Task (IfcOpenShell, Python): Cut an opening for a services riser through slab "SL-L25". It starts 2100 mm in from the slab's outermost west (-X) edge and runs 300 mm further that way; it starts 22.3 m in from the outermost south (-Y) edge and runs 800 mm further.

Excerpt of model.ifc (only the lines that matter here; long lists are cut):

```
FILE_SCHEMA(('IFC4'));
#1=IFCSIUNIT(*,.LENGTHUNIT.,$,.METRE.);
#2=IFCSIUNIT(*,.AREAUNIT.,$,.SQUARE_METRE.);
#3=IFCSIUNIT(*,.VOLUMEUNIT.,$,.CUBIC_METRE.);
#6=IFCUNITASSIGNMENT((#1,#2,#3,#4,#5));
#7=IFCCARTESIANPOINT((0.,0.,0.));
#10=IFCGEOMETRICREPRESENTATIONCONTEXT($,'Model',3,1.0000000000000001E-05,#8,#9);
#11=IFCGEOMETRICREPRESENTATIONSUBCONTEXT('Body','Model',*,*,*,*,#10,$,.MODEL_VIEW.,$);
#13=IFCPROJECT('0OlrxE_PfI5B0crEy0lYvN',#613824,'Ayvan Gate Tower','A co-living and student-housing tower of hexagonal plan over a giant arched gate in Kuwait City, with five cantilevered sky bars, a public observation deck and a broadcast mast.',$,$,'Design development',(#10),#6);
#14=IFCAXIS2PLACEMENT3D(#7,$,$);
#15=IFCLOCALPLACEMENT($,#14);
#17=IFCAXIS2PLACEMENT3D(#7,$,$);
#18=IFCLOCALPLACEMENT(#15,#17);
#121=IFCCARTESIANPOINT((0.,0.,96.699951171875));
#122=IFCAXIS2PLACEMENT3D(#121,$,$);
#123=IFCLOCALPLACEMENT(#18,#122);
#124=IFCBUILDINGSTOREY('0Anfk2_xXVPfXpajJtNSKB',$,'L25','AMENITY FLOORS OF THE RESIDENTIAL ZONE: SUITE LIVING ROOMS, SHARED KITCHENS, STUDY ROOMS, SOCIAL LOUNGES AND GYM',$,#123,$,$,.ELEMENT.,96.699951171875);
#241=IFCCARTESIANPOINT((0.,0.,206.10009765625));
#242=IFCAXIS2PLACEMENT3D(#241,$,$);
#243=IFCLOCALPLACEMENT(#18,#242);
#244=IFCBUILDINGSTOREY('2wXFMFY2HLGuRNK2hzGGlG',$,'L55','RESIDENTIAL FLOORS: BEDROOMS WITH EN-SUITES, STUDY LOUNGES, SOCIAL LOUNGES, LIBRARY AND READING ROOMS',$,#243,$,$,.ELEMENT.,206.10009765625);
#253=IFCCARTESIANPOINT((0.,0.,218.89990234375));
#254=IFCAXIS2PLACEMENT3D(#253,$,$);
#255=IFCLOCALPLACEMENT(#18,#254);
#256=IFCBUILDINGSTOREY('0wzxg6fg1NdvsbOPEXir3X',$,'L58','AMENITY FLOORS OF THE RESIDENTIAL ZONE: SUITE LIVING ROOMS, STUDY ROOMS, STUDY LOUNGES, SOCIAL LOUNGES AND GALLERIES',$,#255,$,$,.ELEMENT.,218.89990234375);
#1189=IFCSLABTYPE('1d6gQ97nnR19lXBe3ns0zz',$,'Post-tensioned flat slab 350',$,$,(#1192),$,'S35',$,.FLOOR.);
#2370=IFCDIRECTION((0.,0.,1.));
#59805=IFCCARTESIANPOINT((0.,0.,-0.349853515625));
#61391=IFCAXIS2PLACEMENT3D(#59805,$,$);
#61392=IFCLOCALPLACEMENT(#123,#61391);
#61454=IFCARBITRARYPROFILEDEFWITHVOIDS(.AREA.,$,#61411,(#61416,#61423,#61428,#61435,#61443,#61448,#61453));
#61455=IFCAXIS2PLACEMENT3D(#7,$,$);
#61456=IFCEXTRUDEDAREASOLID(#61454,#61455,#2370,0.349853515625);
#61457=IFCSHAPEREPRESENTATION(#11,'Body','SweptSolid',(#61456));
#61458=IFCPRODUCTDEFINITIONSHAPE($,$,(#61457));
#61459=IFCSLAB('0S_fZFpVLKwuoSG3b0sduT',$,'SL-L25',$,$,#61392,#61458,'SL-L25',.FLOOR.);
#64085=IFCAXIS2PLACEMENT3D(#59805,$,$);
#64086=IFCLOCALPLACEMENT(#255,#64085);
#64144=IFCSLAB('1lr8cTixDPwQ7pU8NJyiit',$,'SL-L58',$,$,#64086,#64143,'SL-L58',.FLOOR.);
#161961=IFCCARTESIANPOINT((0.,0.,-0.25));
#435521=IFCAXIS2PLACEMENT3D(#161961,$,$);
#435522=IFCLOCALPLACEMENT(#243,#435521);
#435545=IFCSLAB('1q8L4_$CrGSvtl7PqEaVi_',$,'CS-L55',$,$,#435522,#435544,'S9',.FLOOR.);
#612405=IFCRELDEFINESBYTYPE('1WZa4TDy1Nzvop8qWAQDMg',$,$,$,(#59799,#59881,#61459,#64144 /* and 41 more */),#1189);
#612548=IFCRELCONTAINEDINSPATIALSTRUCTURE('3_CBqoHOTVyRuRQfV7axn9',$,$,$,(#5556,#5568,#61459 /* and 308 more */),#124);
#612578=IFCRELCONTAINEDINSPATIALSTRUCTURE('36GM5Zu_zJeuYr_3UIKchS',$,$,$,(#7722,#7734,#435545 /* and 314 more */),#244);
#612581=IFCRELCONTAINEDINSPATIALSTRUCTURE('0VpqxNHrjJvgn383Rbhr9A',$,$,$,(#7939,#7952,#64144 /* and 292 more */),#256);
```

```python
import numpy as np
import ifcopenshell
import ifcopenshell.api.feature
import ifcopenshell.api.geometry
import ifcopenshell.api.root
import ifcopenshell.geom
import ifcopenshell.util.placement
import ifcopenshell.util.representation
import ifcopenshell.util.shape
import ifcopenshell.util.unit

model = ifcopenshell.open("model.ifc")
unit_scale = ifcopenshell.util.unit.calculate_unit_scale(model)
settings = ifcopenshell.geom.settings()


def volume(element):
    """Net volume in cubic metres, openings subtracted."""
    shape = ifcopenshell.geom.create_shape(settings, element)
    return ifcopenshell.util.shape.get_volume(shape.geometry)


slab = model.by_id(61459)
before = volume(slab)

# Extent in the slab's own axes, in metres. The edges named are its -X and -Y sides.
slab_shape = ifcopenshell.geom.create_shape(settings, slab)
vertices = ifcopenshell.util.shape.get_vertices(slab_shape.geometry)
x_min, y_min, bottom = vertices.min(axis=0)
top = vertices[:, 2].max()

opening = ifcopenshell.api.root.create_entity(model, ifc_class="IfcOpeningElement", name="Services riser opening", predefined_type="OPENING")
context = ifcopenshell.util.representation.get_context(model, "Model", "Body", "MODEL_VIEW")
width, depth = 0.3, 0.8
outline = [(0.0, 0.0), (width, 0.0), (width, depth), (0.0, depth), (0.0, 0.0)]
# Overshoot both faces by 50 mm so the cut is clean.
shape = ifcopenshell.api.geometry.add_slab_representation(
    model, context=context, depth=top - bottom + 0.1, polyline=outline
)
ifcopenshell.api.geometry.assign_representation(model, product=opening, representation=shape)

matrix = ifcopenshell.util.placement.get_local_placement(slab.ObjectPlacement)
matrix[:, 3] = matrix @ np.append(np.array([x_min + 2.1, y_min + 22.3, bottom - 0.05]) / unit_scale, 1.0)
ifcopenshell.api.geometry.edit_object_placement(model, product=opening, matrix=matrix, is_si=False)
ifcopenshell.api.feature.add_feature(model, feature=opening, element=slab)

after = volume(slab)

print(f"slab volume {before:.3f} -> {after:.3f} m3")

model.write("model_updated.ifc")
```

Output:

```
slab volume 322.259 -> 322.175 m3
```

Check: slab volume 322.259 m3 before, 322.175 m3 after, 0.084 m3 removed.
